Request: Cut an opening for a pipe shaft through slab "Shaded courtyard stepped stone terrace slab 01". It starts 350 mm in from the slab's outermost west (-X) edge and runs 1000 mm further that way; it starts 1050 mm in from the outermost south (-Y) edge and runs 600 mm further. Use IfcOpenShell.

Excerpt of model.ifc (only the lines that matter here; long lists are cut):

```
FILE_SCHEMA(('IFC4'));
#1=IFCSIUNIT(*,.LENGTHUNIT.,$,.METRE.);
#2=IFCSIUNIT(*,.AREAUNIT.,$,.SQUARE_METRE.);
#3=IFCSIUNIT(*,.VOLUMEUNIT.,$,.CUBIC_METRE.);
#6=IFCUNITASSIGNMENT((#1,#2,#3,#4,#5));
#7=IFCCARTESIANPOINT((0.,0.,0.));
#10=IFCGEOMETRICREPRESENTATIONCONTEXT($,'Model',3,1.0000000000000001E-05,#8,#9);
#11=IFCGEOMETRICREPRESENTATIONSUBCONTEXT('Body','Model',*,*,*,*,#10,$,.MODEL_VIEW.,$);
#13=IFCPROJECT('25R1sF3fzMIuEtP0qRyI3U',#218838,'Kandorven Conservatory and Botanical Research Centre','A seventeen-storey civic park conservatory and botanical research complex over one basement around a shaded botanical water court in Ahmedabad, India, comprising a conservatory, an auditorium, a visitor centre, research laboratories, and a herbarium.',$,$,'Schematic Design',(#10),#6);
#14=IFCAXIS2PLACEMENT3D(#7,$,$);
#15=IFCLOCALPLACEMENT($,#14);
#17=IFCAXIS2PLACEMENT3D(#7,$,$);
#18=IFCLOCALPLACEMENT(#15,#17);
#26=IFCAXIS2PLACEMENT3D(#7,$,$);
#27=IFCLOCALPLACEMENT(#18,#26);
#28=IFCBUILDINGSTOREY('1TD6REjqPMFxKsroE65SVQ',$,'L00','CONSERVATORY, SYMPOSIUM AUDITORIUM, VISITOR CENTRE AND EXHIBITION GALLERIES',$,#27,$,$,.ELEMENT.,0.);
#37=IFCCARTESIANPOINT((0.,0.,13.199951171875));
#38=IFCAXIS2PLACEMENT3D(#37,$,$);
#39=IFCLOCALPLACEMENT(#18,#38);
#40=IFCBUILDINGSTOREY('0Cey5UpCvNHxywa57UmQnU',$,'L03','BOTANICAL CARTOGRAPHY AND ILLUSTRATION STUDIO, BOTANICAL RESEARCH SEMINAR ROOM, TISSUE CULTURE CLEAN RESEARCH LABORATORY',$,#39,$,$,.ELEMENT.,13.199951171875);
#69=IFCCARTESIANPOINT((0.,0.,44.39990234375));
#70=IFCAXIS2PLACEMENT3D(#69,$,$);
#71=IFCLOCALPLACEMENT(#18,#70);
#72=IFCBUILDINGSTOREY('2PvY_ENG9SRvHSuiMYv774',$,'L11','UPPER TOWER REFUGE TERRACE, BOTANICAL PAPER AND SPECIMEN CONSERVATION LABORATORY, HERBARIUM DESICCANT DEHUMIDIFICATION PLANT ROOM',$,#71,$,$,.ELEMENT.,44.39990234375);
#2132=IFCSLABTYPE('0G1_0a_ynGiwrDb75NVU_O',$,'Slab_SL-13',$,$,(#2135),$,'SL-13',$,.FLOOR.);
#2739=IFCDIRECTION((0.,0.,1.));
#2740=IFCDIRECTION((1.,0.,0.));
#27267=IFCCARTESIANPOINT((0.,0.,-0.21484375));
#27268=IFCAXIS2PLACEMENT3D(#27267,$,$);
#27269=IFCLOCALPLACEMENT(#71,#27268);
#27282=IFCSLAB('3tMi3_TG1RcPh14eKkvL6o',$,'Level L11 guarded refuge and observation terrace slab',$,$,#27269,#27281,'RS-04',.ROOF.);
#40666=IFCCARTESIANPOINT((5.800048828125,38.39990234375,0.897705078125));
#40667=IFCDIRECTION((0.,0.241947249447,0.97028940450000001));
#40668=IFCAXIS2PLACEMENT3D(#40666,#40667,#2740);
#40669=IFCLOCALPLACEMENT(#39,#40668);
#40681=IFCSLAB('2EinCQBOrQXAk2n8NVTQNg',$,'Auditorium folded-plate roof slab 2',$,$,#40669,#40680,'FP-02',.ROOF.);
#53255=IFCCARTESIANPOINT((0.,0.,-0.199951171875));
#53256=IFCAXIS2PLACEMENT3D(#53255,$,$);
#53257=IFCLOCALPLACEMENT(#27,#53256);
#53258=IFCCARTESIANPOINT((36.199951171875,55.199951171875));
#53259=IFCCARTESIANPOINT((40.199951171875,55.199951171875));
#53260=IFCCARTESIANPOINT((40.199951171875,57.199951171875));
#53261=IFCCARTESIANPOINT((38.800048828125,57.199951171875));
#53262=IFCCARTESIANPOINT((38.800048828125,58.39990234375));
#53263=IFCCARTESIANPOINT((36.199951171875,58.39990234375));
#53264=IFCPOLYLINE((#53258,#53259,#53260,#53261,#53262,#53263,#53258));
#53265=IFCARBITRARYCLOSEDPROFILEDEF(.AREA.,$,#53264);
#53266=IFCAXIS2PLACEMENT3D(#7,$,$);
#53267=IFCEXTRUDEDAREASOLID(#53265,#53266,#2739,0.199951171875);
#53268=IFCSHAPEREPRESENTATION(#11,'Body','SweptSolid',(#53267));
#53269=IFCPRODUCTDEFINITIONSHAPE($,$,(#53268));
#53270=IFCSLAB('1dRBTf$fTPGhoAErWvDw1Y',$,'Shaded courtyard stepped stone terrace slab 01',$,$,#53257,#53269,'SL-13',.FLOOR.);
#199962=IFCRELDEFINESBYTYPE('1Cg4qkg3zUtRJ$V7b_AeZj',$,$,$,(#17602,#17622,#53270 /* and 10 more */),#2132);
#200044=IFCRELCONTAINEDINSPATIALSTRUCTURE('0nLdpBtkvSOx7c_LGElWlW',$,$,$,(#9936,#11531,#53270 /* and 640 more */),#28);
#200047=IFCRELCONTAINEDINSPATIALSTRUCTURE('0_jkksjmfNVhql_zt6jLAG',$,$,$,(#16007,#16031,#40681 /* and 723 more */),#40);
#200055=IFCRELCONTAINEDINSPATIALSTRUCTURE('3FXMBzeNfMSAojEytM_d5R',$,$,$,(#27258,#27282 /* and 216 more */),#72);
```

```python
import numpy as np
import ifcopenshell
import ifcopenshell.api.feature
import ifcopenshell.api.geometry
import ifcopenshell.api.root
import ifcopenshell.geom
import ifcopenshell.util.placement
import ifcopenshell.util.representation
import ifcopenshell.util.shape
import ifcopenshell.util.unit

model = ifcopenshell.open("model.ifc")
unit_scale = ifcopenshell.util.unit.calculate_unit_scale(model)
settings = ifcopenshell.geom.settings()


def volume(element):
    """Net volume in cubic metres, openings subtracted."""
    shape = ifcopenshell.geom.create_shape(settings, element)
    return ifcopenshell.util.shape.get_volume(shape.geometry)


slab = model.by_guid("1dRBTf$fTPGhoAErWvDw1Y")
before = volume(slab)

# Extent in the slab's own axes, in metres. The edges named are its -X and -Y sides.
slab_shape = ifcopenshell.geom.create_shape(settings, slab)
vertices = ifcopenshell.util.shape.get_vertices(slab_shape.geometry)
x_min, y_min, bottom = vertices.min(axis=0)
top = vertices[:, 2].max()

opening = ifcopenshell.api.root.create_entity(model, ifc_class="IfcOpeningElement", name="Pipe shaft opening", predefined_type="OPENING")
context = ifcopenshell.util.representation.get_context(model, "Model", "Body", "MODEL_VIEW")
width, depth = 1, 0.6
outline = [(0.0, 0.0), (width, 0.0), (width, depth), (0.0, depth), (0.0, 0.0)]
# Overshoot both faces by 50 mm so the cut is clean.
shape = ifcopenshell.api.geometry.add_slab_representation(
    model, context=context, depth=top - bottom + 0.1, polyline=outline
)
ifcopenshell.api.geometry.assign_representation(model, product=opening, representation=shape)

matrix = ifcopenshell.util.placement.get_local_placement(slab.ObjectPlacement)
matrix[:, 3] = matrix @ np.append(np.array([x_min + 0.35, y_min + 1.05, bottom - 0.05]) / unit_scale, 1.0)
ifcopenshell.api.geometry.edit_object_placement(model, product=opening, matrix=matrix, is_si=False)
ifcopenshell.api.feature.add_feature(model, feature=opening, element=slab)

after = volume(slab)

print(f"slab volume {before:.3f} -> {after:.3f} m3")

model.write("model_edited.ifc")
```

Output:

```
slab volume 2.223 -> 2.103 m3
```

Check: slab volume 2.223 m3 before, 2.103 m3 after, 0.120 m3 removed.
